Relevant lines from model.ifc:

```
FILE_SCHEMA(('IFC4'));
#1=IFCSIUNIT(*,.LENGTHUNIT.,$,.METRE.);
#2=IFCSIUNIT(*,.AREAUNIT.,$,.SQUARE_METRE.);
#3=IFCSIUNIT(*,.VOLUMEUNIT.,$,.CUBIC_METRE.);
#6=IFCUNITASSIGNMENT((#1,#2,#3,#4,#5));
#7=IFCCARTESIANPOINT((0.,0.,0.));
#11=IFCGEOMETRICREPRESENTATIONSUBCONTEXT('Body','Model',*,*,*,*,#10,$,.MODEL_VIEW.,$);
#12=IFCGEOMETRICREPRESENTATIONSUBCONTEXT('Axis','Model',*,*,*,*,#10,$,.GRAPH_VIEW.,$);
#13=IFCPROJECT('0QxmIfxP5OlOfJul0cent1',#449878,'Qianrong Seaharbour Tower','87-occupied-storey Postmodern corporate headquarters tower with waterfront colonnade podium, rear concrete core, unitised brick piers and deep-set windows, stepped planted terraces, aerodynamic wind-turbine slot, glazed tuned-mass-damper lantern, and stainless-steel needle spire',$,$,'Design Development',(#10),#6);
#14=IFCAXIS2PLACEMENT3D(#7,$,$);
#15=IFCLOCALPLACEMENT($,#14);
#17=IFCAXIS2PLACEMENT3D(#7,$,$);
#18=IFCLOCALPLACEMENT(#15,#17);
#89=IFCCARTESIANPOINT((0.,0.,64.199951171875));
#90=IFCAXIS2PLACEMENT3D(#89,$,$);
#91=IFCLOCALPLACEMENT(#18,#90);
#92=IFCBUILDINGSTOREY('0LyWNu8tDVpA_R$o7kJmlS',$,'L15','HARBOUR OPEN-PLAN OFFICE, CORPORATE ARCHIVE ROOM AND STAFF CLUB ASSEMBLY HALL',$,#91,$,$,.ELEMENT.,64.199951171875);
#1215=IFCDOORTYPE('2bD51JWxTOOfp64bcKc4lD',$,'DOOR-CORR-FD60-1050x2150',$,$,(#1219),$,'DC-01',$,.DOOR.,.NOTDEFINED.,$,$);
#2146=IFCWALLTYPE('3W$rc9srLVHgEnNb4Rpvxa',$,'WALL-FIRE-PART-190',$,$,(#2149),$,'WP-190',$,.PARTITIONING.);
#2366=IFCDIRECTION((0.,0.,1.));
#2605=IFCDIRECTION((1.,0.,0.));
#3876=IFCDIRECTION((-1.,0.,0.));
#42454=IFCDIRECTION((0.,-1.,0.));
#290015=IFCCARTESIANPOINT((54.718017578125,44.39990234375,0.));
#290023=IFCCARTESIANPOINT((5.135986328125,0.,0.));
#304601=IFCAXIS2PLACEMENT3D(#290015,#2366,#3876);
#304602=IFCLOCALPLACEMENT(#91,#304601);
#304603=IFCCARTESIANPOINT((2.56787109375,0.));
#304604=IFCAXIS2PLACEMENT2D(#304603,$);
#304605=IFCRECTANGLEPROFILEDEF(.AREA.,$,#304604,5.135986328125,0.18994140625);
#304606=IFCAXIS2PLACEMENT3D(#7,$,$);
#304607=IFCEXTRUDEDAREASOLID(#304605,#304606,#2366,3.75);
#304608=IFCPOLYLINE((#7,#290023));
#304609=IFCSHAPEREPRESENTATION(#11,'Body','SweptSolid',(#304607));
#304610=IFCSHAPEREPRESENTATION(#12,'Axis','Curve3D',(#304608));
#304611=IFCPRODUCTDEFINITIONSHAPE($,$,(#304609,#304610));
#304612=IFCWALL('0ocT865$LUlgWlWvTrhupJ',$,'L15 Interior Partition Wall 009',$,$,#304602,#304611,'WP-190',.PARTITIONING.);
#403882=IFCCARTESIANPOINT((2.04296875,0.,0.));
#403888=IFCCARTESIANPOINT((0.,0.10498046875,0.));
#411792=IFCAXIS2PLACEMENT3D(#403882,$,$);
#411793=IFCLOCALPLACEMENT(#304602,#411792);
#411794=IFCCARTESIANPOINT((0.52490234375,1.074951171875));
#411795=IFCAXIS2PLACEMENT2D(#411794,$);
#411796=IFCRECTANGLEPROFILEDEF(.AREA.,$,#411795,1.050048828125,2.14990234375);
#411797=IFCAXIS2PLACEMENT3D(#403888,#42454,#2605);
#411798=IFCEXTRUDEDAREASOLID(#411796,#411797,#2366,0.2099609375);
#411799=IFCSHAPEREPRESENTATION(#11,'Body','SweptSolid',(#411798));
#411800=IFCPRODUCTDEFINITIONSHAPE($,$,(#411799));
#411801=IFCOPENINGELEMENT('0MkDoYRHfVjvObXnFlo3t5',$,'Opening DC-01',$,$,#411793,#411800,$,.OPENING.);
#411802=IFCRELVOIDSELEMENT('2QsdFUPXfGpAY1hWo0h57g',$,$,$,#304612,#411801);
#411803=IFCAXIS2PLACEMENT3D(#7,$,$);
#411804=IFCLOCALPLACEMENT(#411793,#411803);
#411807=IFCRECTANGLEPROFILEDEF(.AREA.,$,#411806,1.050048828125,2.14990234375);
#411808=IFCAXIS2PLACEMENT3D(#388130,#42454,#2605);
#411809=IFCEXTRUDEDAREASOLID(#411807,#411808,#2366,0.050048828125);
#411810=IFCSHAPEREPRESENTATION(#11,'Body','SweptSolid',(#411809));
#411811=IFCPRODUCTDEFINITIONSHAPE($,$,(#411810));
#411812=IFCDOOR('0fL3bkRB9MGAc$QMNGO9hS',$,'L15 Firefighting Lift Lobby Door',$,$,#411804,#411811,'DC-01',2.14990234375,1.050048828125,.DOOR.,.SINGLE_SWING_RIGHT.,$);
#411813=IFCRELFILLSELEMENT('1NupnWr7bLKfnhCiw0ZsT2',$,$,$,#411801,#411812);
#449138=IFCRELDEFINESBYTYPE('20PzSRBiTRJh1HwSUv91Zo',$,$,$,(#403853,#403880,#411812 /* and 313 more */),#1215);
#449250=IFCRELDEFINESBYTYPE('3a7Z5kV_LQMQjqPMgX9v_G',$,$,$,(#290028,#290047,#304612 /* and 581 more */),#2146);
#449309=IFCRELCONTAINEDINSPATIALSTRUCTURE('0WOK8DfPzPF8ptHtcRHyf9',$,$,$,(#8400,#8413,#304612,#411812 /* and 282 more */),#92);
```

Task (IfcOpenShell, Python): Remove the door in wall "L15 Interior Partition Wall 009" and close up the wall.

```python
import ifcopenshell
import ifcopenshell.api.feature
import ifcopenshell.api.root
import ifcopenshell.geom
import ifcopenshell.util.shape

model = ifcopenshell.open("model.ifc")
settings = ifcopenshell.geom.settings()


def volume(element):
    """Net volume in cubic metres, openings subtracted."""
    shape = ifcopenshell.geom.create_shape(settings, element)
    return ifcopenshell.util.shape.get_volume(shape.geometry)


door = model.by_id(411812)
opening = door.FillsVoids[0].RelatingOpeningElement
wall = opening.VoidsElements[0].RelatingBuildingElement
before = volume(wall)

ifcopenshell.api.root.remove_product(model, product=door)
ifcopenshell.api.feature.remove_feature(model, feature=opening)

after = volume(wall)

print(f"wall volume {before:.3f} -> {after:.3f} m3")

model.write("model_v2.ifc")
```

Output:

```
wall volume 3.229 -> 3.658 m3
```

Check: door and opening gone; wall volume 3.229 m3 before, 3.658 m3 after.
